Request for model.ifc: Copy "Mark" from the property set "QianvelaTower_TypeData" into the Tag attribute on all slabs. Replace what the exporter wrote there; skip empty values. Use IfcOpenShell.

First a look at what the model holds.

```python
import ifcopenshell
import ifcopenshell.util.element

model = ifcopenshell.open("model.ifc")
print(model.schema)
slabs = model.by_type("IfcSlab")
print(len(slabs), "slabs")
for e in slabs[:8]:
    source = ifcopenshell.util.element.get_pset(e, "QianvelaTower_TypeData", "Mark")
    target = e.Tag
    print(e.id(), repr(source), repr(target), sep=" | ")
```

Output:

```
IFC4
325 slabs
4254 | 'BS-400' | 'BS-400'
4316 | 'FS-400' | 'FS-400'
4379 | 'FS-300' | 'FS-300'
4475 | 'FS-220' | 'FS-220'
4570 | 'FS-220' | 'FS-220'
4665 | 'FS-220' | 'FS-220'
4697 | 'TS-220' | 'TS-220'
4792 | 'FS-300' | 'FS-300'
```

```python
import ifcopenshell
import ifcopenshell.util.element

model = ifcopenshell.open("model.ifc")

count = 0
for e in model.by_type("IfcSlab"):
    value = ifcopenshell.util.element.get_pset(e, "QianvelaTower_TypeData", "Mark")
    current = e.Tag
    if not value or not value.strip() or current == value:
        continue
    e.Tag = value
    count += 1

print(count, "slabs updated")

model.write("model_v2.ifc")
```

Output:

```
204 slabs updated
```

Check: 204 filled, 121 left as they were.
